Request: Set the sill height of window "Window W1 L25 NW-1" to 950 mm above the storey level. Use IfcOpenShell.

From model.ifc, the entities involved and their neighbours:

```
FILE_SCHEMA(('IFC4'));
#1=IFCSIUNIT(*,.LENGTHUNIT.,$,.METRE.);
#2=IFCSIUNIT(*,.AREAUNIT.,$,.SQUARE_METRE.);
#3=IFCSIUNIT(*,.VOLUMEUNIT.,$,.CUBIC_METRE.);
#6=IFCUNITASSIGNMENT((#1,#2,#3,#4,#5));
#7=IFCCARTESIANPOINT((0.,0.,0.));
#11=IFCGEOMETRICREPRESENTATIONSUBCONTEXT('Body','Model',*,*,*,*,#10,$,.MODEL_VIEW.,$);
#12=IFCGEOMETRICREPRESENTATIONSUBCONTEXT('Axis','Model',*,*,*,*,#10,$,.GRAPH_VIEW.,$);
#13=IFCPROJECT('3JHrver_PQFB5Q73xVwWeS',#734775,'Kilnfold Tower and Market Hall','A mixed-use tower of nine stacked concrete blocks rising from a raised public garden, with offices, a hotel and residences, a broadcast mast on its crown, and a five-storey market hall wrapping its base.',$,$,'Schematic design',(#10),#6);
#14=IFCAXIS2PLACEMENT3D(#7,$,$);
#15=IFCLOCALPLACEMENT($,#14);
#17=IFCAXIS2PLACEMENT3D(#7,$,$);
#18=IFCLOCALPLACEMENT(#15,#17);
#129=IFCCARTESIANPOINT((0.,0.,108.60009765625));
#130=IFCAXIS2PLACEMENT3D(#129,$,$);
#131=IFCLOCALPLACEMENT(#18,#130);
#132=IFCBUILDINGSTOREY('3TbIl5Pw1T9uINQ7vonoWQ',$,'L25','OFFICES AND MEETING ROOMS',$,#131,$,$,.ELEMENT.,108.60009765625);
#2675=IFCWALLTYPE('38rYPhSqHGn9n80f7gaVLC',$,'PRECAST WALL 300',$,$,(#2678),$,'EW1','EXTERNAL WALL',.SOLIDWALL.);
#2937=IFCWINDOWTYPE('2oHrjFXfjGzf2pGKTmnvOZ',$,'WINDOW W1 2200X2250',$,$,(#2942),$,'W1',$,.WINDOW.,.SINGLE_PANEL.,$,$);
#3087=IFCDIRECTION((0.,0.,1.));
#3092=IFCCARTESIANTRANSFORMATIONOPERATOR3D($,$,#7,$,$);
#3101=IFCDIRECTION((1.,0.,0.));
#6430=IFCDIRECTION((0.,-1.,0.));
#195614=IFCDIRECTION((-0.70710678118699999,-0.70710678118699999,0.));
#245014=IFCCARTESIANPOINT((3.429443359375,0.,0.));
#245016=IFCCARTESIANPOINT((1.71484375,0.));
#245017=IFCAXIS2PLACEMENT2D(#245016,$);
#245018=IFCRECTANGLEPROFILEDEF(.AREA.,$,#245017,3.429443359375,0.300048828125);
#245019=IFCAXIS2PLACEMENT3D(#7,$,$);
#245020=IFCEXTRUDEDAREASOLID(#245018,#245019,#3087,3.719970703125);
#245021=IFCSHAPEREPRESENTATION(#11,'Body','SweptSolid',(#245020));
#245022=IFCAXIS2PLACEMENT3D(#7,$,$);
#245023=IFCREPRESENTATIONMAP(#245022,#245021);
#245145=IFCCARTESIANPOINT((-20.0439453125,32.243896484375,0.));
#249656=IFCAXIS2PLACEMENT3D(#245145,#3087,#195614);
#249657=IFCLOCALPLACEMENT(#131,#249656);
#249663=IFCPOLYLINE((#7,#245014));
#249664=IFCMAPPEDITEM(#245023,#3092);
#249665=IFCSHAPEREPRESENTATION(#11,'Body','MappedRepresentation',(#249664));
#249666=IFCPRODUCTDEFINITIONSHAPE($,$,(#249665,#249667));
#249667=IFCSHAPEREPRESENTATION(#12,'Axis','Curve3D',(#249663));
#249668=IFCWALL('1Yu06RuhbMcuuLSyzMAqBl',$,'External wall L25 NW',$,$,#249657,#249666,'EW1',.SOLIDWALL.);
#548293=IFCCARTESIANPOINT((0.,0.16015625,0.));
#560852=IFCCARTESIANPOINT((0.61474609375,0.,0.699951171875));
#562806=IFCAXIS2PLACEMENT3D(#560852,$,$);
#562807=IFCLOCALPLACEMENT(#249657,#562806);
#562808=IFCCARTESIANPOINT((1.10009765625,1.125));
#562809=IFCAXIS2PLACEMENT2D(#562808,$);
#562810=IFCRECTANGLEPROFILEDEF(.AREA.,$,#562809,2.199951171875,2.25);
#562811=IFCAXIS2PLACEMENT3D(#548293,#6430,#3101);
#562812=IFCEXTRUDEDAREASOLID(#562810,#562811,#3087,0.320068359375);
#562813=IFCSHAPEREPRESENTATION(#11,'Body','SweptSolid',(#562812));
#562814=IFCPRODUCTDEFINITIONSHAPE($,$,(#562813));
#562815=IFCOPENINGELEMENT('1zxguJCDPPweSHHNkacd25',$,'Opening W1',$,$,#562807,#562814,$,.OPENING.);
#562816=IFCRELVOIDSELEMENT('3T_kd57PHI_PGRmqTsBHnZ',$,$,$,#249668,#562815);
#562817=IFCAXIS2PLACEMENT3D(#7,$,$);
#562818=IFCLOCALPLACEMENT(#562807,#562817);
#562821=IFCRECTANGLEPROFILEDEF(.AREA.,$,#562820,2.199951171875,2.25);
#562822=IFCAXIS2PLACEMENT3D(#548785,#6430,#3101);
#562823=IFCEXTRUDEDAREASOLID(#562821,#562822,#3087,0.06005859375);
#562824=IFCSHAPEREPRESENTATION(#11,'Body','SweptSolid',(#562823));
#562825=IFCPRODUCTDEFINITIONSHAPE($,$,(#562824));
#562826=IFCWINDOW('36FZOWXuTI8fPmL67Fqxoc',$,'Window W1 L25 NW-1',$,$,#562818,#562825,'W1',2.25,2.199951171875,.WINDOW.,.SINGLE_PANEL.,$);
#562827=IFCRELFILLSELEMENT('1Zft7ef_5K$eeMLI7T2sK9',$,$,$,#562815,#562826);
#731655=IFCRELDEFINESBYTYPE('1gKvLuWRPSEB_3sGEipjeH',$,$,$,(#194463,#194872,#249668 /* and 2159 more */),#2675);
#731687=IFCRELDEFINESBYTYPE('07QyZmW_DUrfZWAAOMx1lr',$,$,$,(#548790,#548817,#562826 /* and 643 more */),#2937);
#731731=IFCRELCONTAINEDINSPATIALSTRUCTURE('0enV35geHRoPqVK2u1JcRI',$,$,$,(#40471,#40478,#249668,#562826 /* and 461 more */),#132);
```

```python
import numpy as np
import ifcopenshell
import ifcopenshell.api.geometry
import ifcopenshell.geom
import ifcopenshell.util.element
import ifcopenshell.util.placement
import ifcopenshell.util.shape
import ifcopenshell.util.unit

model = ifcopenshell.open("model.ifc")
unit_scale = ifcopenshell.util.unit.calculate_unit_scale(model)

window = model.by_guid("36FZOWXuTI8fPmL67Fqxoc")
opening = window.FillsVoids[0].RelatingOpeningElement
storey = ifcopenshell.util.element.get_container(window, ifc_class="IfcBuildingStorey")
level = ifcopenshell.util.placement.get_local_placement(storey.ObjectPlacement)[2, 3]

# The opening's origin need not be at the sill, so measure its lowest point.
shape = ifcopenshell.geom.create_shape(ifcopenshell.geom.settings(), opening)
bottom = ifcopenshell.util.shape.get_shape_bottom_elevation(shape, shape.geometry) / unit_scale
dz = level + 0.95 / unit_scale - bottom

shift = np.array([0.0, 0.0, dz])
# The window is placed relative to its opening, so it follows when the opening moves.
matrix = ifcopenshell.util.placement.get_local_placement(opening.ObjectPlacement)
matrix[:3, 3] += shift
ifcopenshell.api.geometry.edit_object_placement(
    model, product=opening, matrix=matrix, is_si=False, should_transform_children=True
)

print(f"moved by {dz * unit_scale:+.3f} m")

model.write("model_v2.ifc")
```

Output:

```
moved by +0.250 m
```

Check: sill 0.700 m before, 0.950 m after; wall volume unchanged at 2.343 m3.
